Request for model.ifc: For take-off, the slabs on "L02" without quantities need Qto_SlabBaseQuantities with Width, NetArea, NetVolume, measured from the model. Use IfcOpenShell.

First a look at what the model holds.

```python
import ifcopenshell
import ifcopenshell.util.element
import ifcopenshell.util.unit

model = ifcopenshell.open("model.ifc")
print(model.schema)
for unit_type in ("LENGTHUNIT", "AREAUNIT", "VOLUMEUNIT"):
    print(unit_type, ifcopenshell.util.unit.calculate_unit_scale(model, unit_type))
storey = next(s for s in model.by_type("IfcBuildingStorey") if s.Name == "L02")
slabs = [e for e in ifcopenshell.util.element.get_decomposition(storey) if e.is_a("IfcSlab")]
for e in sorted(slabs, key=lambda e: e.id()):
    print(e.id(), e.is_a(), e.Name, list(ifcopenshell.util.element.get_psets(e, qtos_only=True)), sep=" | ")
```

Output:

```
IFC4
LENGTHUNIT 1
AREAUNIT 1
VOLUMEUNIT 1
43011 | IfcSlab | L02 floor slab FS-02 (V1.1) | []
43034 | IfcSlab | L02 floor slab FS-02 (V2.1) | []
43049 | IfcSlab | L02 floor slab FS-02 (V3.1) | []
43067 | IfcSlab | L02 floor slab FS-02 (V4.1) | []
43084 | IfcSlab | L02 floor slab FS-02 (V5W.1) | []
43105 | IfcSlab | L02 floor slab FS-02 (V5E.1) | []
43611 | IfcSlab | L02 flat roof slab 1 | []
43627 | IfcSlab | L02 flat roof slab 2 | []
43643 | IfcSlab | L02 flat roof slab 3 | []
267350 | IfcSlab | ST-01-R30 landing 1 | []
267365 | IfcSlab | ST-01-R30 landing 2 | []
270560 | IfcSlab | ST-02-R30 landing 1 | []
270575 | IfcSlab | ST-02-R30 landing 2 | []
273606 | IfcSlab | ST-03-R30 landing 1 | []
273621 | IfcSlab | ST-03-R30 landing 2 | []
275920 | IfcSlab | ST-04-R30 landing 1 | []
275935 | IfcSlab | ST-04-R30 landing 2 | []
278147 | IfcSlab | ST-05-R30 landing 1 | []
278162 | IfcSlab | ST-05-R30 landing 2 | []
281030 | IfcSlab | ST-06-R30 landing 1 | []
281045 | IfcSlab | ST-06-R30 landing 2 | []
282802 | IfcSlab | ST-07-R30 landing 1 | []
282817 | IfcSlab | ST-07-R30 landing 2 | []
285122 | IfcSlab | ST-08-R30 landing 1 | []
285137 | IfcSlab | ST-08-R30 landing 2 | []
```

```python
import ifcopenshell
import ifcopenshell.api.pset
import ifcopenshell.geom
import ifcopenshell.util.element
import ifcopenshell.util.shape
import ifcopenshell.util.unit

model = ifcopenshell.open("model.ifc")
unit_scale = ifcopenshell.util.unit.calculate_unit_scale(model)
area_scale = ifcopenshell.util.unit.calculate_unit_scale(model, "AREAUNIT")
volume_scale = ifcopenshell.util.unit.calculate_unit_scale(model, "VOLUMEUNIT")
settings = ifcopenshell.geom.settings()

storey = next(s for s in model.by_type("IfcBuildingStorey") if s.Name == "L02")
slabs = [e for e in ifcopenshell.util.element.get_decomposition(storey) if e.is_a("IfcSlab")]

for e in sorted(slabs, key=lambda e: e.id()):
    if ifcopenshell.util.element.get_psets(e, qtos_only=True, should_inherit=False):
        continue
    # Geometry comes back in metres, in the element's own axes.
    shape = ifcopenshell.geom.create_shape(settings, e)
    values = {
        "Width": ifcopenshell.util.shape.get_z(shape.geometry) / unit_scale,
        "NetArea": ifcopenshell.util.shape.get_footprint_area(shape.geometry) / area_scale,
        "NetVolume": ifcopenshell.util.shape.get_volume(shape.geometry) / volume_scale,
    }
    qto = ifcopenshell.api.pset.add_qto(model, product=e, name="Qto_SlabBaseQuantities")
    ifcopenshell.api.pset.edit_qto(model, qto=qto, properties=values)
    print(e.id(), {k: round(v, 3) for k, v in values.items()})

model.write("model-out.ifc")
```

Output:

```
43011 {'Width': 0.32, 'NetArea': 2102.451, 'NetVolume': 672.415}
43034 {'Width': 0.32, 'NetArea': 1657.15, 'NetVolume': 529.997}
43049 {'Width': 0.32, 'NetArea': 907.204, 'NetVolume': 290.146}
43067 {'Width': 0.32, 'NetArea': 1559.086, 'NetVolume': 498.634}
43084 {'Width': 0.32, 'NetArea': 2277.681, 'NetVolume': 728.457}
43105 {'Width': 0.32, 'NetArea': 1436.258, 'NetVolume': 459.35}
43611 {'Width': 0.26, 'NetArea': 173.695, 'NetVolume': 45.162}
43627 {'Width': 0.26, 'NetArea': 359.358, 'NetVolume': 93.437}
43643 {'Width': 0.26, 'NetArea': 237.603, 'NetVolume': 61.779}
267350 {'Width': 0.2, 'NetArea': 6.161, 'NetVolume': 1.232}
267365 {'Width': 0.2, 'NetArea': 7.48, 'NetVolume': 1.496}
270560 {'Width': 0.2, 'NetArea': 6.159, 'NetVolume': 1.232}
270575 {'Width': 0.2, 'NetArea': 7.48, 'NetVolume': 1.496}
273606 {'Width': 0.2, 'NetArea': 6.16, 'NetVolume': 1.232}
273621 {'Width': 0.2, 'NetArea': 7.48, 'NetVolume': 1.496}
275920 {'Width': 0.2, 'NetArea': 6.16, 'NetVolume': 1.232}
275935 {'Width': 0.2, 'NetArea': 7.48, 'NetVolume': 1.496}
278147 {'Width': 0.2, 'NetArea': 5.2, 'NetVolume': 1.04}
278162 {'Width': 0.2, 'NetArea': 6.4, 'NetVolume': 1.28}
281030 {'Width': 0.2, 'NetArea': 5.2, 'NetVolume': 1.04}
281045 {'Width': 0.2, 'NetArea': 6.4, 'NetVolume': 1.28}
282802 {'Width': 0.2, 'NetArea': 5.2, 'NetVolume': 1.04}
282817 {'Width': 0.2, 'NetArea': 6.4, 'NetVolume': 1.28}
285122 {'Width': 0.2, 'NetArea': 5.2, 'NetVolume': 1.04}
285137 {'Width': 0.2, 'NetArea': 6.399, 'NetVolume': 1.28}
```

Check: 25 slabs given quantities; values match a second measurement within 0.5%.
